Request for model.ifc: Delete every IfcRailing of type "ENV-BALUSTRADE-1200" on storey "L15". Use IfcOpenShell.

First a look at what the model holds.

```python
import ifcopenshell
import ifcopenshell.util.element

model = ifcopenshell.open("model.ifc")
print(model.schema)
storey = next(s for s in model.by_type("IfcBuildingStorey") if s.Name == "L15")
railings = [e for e in ifcopenshell.util.element.get_decomposition(storey) if e.is_a("IfcRailing")]
seen = {}
for e in railings:
    element_type = ifcopenshell.util.element.get_type(e)
    name = element_type.Name if element_type not in (None, e) else None
    seen[name] = seen.get(name, 0) + 1
for name, count in sorted(seen.items(), key=str):
    print(count, "x", name)
```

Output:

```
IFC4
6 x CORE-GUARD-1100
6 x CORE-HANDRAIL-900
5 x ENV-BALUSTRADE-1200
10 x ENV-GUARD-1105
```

```python
import ifcopenshell
import ifcopenshell.api.root
import ifcopenshell.util.element

model = ifcopenshell.open("model.ifc")

storey = next(s for s in model.by_type("IfcBuildingStorey") if s.Name == "L15")
railings = [e for e in ifcopenshell.util.element.get_decomposition(storey) if e.is_a("IfcRailing")]
targets = [e for e in railings if (t := ifcopenshell.util.element.get_type(e)) not in (None, e) and t.Name == "ENV-BALUSTRADE-1200"]

for e in targets:
    ifcopenshell.api.root.remove_product(model, product=e)
print(len(targets), "removed")

model.write("model_updated.ifc")
```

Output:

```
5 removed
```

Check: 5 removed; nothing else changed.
